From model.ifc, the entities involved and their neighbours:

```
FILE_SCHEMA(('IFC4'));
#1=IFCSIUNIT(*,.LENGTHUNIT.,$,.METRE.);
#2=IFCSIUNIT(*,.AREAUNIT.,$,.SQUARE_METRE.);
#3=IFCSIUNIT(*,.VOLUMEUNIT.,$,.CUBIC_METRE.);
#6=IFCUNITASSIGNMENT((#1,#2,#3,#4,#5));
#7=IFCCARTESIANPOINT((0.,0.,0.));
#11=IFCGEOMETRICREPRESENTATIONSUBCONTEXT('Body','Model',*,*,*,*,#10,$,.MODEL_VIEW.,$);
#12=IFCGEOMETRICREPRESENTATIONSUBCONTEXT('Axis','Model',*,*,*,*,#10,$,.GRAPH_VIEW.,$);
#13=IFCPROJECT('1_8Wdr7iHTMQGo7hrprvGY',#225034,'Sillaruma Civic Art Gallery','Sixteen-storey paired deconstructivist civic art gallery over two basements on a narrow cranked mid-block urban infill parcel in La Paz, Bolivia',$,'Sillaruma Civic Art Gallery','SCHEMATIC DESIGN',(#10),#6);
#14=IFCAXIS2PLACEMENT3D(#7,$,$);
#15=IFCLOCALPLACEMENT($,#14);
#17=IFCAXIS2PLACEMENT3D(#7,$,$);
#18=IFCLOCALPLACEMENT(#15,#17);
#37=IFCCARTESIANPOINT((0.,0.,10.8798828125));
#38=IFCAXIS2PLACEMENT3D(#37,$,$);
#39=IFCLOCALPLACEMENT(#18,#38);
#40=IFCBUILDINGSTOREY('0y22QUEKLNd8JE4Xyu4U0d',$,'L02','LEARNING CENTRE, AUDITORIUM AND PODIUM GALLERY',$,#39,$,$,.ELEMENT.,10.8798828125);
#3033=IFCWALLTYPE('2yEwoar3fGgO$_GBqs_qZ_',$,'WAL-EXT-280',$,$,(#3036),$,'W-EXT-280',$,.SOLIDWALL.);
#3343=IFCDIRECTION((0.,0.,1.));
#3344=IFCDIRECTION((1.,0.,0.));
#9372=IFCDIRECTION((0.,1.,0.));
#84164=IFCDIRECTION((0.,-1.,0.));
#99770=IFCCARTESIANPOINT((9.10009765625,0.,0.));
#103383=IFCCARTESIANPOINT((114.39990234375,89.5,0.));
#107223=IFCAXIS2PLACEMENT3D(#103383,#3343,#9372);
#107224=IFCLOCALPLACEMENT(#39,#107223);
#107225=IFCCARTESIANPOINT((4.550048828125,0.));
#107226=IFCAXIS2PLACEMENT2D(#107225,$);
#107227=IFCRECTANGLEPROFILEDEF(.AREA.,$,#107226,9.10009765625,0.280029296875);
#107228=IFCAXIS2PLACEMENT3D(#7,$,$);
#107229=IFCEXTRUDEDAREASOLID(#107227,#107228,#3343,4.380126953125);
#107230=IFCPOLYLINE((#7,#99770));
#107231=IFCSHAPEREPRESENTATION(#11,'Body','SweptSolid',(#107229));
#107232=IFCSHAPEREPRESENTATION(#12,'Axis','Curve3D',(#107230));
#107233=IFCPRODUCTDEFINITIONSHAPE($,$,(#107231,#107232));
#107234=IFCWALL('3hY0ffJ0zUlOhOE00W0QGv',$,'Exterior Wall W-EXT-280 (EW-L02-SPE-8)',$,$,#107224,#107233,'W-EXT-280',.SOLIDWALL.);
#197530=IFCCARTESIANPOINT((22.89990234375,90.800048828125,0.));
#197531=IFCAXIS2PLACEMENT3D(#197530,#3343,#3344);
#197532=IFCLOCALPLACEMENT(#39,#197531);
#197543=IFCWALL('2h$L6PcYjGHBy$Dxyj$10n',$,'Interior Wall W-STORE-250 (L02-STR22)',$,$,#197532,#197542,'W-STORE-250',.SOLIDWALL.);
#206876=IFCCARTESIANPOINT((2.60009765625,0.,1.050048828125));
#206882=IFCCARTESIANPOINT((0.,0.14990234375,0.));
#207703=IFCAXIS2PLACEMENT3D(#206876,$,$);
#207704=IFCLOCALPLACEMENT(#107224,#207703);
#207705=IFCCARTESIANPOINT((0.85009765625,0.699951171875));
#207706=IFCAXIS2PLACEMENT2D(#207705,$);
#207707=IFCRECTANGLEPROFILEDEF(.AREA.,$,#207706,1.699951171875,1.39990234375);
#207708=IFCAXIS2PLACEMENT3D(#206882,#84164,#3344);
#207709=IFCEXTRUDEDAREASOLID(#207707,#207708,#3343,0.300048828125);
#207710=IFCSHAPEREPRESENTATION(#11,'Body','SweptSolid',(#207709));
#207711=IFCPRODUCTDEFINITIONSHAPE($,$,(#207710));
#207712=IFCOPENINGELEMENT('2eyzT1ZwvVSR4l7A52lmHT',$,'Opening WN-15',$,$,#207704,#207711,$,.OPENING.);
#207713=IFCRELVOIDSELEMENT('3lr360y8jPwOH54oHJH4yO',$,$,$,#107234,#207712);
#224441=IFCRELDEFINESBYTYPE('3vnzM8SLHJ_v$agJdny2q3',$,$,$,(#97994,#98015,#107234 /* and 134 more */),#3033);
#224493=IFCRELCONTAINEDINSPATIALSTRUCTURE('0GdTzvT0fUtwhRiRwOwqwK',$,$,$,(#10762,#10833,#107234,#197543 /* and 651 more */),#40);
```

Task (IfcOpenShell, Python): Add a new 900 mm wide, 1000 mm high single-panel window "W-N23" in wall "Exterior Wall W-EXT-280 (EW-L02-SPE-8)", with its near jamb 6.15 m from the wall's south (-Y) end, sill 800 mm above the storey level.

```python
import numpy as np
import ifcopenshell
import ifcopenshell.api.feature
import ifcopenshell.api.geometry
import ifcopenshell.api.root
import ifcopenshell.api.spatial
import ifcopenshell.geom
import ifcopenshell.util.element
import ifcopenshell.util.placement
import ifcopenshell.util.representation
import ifcopenshell.util.shape
import ifcopenshell.util.unit

model = ifcopenshell.open("model.ifc")
unit_scale = ifcopenshell.util.unit.calculate_unit_scale(model)
settings = ifcopenshell.geom.settings()


def volume(element):
    """Net volume in cubic metres, openings subtracted."""
    shape = ifcopenshell.geom.create_shape(settings, element)
    return ifcopenshell.util.shape.get_volume(shape.geometry)


wall = model.by_id(107234)
storey = ifcopenshell.util.element.get_container(wall, ifc_class="IfcBuildingStorey")
context = ifcopenshell.util.representation.get_context(model, "Model", "Body", "MODEL_VIEW")
before = volume(wall)

width, height, from_end, sill = 0.9, 1, 6.15, 0.8  # metres

# The wall runs along its own X axis, and the end named is its -X end.
wall_shape = ifcopenshell.geom.create_shape(settings, wall)
x, y, z = ifcopenshell.util.shape.get_vertices(wall_shape.geometry).T
start = x.min() + from_end
face, thickness = float(y.min()), float(y.max() - y.min())
wall_matrix = ifcopenshell.util.placement.get_local_placement(wall.ObjectPlacement)
level = ifcopenshell.util.placement.get_local_placement(storey.ObjectPlacement)[2, 3]


def in_wall(x, y):
    """Placement at x, y metres in the wall's axes, at sill height."""
    matrix = wall_matrix.copy()
    matrix[:, 3] = wall_matrix @ np.array([x / unit_scale, y / unit_scale, 0.0, 1.0])
    matrix[2, 3] = level + sill / unit_scale
    return matrix


# Opening: a box that overshoots both wall faces by 50 mm.
opening = ifcopenshell.api.root.create_entity(model, ifc_class="IfcOpeningElement", predefined_type="OPENING")
box = ifcopenshell.api.geometry.add_wall_representation(
    model, context=context, length=width, height=height, thickness=thickness + 0.1
)
ifcopenshell.api.geometry.assign_representation(model, product=opening, representation=box)
ifcopenshell.api.geometry.edit_object_placement(model, product=opening, matrix=in_wall(start, face - 0.05), is_si=False)
ifcopenshell.api.feature.add_feature(model, feature=opening, element=wall)

window = ifcopenshell.api.root.create_entity(model, ifc_class="IfcWindow", name="W-N23", predefined_type="WINDOW")
window.OverallWidth, window.OverallHeight = width / unit_scale, height / unit_scale
window.PartitioningType = "SINGLE_PANEL"
body = ifcopenshell.api.geometry.add_window_representation(
    model,
    context=context,
    overall_width=window.OverallWidth,
    overall_height=window.OverallHeight,
    partition_type="SINGLE_PANEL",
)
ifcopenshell.api.geometry.assign_representation(model, product=window, representation=body)
ifcopenshell.api.spatial.assign_container(model, products=[window], relating_structure=storey)
ifcopenshell.api.feature.add_filling(model, opening=opening, element=window)

# Centre the window in the wall's thickness.
ifcopenshell.api.geometry.edit_object_placement(model, product=window, matrix=in_wall(start, face), is_si=False)
window_shape = ifcopenshell.geom.create_shape(settings, window)
depth = ifcopenshell.util.shape.get_vertices(window_shape.geometry)[:, 1]
offset = face + thickness / 2 - (depth.min() + depth.max()) / 2
ifcopenshell.api.geometry.edit_object_placement(model, product=window, matrix=in_wall(start, offset), is_si=False)

after = volume(wall)

print(f"wall volume {before:.3f} -> {after:.3f} m3")

model.write("model_rev.ifc")
```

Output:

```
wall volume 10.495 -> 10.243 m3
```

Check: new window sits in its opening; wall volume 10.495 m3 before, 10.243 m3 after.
